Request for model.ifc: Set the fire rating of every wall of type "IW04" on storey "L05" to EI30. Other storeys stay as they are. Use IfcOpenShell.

First a look at what the model holds.

```python
import ifcopenshell
import ifcopenshell.util.element

model = ifcopenshell.open("model.ifc")
print(model.schema)
storey = next(s for s in model.by_type("IfcBuildingStorey") if s.Name == "L05")
walls = [e for e in ifcopenshell.util.element.get_decomposition(storey) if e.is_a("IfcWall")]
seen = {}
for e in walls:
    element_type = ifcopenshell.util.element.get_type(e)
    key = (element_type.Name if element_type != e and element_type else None, ifcopenshell.util.element.get_pset(e, "Pset_WallCommon", "FireRating"))
    seen[key] = seen.get(key, 0) + 1
for (name, value), count in sorted(seen.items(), key=str):
    print(count, "x", name, "|", value)
```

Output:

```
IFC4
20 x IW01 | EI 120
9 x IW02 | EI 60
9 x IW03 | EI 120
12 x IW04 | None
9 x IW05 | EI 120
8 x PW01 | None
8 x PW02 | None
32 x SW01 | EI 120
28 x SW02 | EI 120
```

```python
import ifcopenshell
import ifcopenshell.api.pset
import ifcopenshell.util.element

model = ifcopenshell.open("model.ifc")

storey = next(s for s in model.by_type("IfcBuildingStorey") if s.Name == "L05")
walls = [e for e in ifcopenshell.util.element.get_decomposition(storey) if e.is_a("IfcWall")]

count = 0
for e in walls:
    element_type = ifcopenshell.util.element.get_type(e)
    if element_type in (None, e) or element_type.Name != "IW04":
        continue
    # add_pset returns the element's existing set when there is one.
    pset = ifcopenshell.api.pset.add_pset(model, product=e, name="Pset_WallCommon")
    ifcopenshell.api.pset.edit_pset(model, pset=pset, properties={"FireRating": "EI30"})
    count += 1

print(count, "walls updated")

model.write("model_v2.ifc")
```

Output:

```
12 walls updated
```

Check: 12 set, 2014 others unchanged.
